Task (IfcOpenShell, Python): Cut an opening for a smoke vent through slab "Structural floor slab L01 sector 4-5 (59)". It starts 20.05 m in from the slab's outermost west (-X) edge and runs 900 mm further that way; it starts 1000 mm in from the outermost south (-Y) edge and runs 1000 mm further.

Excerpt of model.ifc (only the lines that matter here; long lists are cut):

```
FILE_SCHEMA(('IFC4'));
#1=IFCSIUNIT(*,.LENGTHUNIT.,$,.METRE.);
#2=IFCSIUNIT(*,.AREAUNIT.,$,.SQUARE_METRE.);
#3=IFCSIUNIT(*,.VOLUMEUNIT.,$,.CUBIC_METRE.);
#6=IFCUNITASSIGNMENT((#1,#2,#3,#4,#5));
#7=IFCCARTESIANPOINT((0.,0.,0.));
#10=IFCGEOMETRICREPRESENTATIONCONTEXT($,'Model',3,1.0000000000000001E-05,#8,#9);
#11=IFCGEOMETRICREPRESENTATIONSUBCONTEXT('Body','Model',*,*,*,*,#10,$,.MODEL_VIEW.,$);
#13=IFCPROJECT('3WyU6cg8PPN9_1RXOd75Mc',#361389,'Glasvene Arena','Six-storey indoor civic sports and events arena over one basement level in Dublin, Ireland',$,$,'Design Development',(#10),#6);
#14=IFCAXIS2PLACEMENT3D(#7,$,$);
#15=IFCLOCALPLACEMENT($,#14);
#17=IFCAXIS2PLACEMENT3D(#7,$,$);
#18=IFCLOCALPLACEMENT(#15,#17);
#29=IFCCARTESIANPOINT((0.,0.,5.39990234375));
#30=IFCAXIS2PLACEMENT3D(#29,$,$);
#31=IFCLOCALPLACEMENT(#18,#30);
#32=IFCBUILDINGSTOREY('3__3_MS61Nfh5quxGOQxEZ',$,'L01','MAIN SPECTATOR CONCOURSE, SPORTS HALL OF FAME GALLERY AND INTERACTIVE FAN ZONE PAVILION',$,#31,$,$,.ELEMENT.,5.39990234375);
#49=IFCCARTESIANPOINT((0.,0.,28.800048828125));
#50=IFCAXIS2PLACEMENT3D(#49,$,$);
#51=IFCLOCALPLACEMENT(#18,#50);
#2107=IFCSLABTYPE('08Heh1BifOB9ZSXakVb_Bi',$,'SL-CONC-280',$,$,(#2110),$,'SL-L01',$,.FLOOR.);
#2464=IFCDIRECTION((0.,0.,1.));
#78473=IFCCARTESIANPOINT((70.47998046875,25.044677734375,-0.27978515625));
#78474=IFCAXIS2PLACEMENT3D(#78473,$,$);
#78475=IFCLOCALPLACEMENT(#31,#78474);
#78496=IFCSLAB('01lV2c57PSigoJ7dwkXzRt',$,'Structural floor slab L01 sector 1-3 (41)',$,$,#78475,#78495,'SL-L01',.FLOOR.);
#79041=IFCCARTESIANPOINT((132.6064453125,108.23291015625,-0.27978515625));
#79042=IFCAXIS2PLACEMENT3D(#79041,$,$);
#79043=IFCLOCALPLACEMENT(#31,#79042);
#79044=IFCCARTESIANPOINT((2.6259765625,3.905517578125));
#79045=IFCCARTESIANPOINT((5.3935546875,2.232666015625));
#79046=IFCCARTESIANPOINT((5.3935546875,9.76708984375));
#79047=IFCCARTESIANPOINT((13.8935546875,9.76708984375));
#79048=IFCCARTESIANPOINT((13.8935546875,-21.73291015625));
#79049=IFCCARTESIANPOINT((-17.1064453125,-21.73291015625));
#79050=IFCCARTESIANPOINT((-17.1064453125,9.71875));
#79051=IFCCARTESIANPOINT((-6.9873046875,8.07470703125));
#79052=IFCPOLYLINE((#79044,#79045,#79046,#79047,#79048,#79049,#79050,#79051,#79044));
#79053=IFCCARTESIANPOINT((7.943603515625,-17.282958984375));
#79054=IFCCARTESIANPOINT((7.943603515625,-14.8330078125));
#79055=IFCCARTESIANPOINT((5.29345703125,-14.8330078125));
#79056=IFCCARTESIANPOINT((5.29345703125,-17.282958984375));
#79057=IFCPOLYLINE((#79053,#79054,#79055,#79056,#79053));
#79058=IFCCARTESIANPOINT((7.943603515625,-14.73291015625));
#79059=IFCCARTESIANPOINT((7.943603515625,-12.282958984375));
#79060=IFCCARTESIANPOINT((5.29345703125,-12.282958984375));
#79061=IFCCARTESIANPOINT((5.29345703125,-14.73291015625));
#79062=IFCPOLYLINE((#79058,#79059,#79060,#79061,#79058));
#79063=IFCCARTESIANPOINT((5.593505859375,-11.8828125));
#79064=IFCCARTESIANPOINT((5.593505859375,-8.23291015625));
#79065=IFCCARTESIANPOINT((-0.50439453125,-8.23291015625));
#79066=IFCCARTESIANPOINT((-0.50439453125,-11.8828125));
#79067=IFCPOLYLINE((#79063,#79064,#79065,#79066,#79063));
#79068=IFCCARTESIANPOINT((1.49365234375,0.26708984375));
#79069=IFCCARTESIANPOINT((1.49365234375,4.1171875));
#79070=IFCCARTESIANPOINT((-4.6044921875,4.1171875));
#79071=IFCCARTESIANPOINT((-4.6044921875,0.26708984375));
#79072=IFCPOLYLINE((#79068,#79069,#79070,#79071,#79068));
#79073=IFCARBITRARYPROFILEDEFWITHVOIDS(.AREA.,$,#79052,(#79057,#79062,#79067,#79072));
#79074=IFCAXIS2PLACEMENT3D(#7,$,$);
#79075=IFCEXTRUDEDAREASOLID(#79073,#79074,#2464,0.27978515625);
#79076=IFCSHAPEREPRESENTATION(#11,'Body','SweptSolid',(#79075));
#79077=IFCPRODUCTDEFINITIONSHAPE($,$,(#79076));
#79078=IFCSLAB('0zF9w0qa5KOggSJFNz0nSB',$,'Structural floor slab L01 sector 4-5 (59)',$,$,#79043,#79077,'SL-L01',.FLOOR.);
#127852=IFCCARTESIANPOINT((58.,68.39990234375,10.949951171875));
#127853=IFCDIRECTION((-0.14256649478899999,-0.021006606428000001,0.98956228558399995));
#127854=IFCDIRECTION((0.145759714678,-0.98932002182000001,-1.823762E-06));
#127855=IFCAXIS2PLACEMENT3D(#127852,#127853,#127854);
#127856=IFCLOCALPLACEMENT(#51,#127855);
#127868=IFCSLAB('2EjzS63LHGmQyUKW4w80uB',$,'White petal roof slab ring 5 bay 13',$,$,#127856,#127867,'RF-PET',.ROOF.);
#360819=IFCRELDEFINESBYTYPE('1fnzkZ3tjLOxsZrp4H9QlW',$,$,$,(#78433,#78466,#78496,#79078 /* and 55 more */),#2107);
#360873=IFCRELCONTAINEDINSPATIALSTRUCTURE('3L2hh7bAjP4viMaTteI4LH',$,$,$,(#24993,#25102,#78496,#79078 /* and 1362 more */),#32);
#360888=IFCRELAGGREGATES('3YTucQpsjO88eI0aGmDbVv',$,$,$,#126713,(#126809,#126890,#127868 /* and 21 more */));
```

```python
import numpy as np
import ifcopenshell
import ifcopenshell.api.feature
import ifcopenshell.api.geometry
import ifcopenshell.api.root
import ifcopenshell.geom
import ifcopenshell.util.placement
import ifcopenshell.util.representation
import ifcopenshell.util.shape
import ifcopenshell.util.unit

model = ifcopenshell.open("model.ifc")
unit_scale = ifcopenshell.util.unit.calculate_unit_scale(model)
settings = ifcopenshell.geom.settings()


def volume(element):
    """Net volume in cubic metres, openings subtracted."""
    shape = ifcopenshell.geom.create_shape(settings, element)
    return ifcopenshell.util.shape.get_volume(shape.geometry)


slab = model.by_guid("0zF9w0qa5KOggSJFNz0nSB")
before = volume(slab)

# Extent in the slab's own axes, in metres. The edges named are its -X and -Y sides.
slab_shape = ifcopenshell.geom.create_shape(settings, slab)
vertices = ifcopenshell.util.shape.get_vertices(slab_shape.geometry)
x_min, y_min, bottom = vertices.min(axis=0)
top = vertices[:, 2].max()

opening = ifcopenshell.api.root.create_entity(model, ifc_class="IfcOpeningElement", name="Smoke vent opening", predefined_type="OPENING")
context = ifcopenshell.util.representation.get_context(model, "Model", "Body", "MODEL_VIEW")
width, depth = 0.9, 1
outline = [(0.0, 0.0), (width, 0.0), (width, depth), (0.0, depth), (0.0, 0.0)]
# Overshoot both faces by 50 mm so the cut is clean.
shape = ifcopenshell.api.geometry.add_slab_representation(
    model, context=context, depth=top - bottom + 0.1, polyline=outline
)
ifcopenshell.api.geometry.assign_representation(model, product=opening, representation=shape)

matrix = ifcopenshell.util.placement.get_local_placement(slab.ObjectPlacement)
matrix[:, 3] = matrix @ np.append(np.array([x_min + 20.05, y_min + 1, bottom - 0.05]) / unit_scale, 1.0)
ifcopenshell.api.geometry.edit_object_placement(model, product=opening, matrix=matrix, is_si=False)
ifcopenshell.api.feature.add_feature(model, feature=opening, element=slab)

after = volume(slab)

print(f"slab volume {before:.3f} -> {after:.3f} m3")

model.write("model_v2.ifc")
```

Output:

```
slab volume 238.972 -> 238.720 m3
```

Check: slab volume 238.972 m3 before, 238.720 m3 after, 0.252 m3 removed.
